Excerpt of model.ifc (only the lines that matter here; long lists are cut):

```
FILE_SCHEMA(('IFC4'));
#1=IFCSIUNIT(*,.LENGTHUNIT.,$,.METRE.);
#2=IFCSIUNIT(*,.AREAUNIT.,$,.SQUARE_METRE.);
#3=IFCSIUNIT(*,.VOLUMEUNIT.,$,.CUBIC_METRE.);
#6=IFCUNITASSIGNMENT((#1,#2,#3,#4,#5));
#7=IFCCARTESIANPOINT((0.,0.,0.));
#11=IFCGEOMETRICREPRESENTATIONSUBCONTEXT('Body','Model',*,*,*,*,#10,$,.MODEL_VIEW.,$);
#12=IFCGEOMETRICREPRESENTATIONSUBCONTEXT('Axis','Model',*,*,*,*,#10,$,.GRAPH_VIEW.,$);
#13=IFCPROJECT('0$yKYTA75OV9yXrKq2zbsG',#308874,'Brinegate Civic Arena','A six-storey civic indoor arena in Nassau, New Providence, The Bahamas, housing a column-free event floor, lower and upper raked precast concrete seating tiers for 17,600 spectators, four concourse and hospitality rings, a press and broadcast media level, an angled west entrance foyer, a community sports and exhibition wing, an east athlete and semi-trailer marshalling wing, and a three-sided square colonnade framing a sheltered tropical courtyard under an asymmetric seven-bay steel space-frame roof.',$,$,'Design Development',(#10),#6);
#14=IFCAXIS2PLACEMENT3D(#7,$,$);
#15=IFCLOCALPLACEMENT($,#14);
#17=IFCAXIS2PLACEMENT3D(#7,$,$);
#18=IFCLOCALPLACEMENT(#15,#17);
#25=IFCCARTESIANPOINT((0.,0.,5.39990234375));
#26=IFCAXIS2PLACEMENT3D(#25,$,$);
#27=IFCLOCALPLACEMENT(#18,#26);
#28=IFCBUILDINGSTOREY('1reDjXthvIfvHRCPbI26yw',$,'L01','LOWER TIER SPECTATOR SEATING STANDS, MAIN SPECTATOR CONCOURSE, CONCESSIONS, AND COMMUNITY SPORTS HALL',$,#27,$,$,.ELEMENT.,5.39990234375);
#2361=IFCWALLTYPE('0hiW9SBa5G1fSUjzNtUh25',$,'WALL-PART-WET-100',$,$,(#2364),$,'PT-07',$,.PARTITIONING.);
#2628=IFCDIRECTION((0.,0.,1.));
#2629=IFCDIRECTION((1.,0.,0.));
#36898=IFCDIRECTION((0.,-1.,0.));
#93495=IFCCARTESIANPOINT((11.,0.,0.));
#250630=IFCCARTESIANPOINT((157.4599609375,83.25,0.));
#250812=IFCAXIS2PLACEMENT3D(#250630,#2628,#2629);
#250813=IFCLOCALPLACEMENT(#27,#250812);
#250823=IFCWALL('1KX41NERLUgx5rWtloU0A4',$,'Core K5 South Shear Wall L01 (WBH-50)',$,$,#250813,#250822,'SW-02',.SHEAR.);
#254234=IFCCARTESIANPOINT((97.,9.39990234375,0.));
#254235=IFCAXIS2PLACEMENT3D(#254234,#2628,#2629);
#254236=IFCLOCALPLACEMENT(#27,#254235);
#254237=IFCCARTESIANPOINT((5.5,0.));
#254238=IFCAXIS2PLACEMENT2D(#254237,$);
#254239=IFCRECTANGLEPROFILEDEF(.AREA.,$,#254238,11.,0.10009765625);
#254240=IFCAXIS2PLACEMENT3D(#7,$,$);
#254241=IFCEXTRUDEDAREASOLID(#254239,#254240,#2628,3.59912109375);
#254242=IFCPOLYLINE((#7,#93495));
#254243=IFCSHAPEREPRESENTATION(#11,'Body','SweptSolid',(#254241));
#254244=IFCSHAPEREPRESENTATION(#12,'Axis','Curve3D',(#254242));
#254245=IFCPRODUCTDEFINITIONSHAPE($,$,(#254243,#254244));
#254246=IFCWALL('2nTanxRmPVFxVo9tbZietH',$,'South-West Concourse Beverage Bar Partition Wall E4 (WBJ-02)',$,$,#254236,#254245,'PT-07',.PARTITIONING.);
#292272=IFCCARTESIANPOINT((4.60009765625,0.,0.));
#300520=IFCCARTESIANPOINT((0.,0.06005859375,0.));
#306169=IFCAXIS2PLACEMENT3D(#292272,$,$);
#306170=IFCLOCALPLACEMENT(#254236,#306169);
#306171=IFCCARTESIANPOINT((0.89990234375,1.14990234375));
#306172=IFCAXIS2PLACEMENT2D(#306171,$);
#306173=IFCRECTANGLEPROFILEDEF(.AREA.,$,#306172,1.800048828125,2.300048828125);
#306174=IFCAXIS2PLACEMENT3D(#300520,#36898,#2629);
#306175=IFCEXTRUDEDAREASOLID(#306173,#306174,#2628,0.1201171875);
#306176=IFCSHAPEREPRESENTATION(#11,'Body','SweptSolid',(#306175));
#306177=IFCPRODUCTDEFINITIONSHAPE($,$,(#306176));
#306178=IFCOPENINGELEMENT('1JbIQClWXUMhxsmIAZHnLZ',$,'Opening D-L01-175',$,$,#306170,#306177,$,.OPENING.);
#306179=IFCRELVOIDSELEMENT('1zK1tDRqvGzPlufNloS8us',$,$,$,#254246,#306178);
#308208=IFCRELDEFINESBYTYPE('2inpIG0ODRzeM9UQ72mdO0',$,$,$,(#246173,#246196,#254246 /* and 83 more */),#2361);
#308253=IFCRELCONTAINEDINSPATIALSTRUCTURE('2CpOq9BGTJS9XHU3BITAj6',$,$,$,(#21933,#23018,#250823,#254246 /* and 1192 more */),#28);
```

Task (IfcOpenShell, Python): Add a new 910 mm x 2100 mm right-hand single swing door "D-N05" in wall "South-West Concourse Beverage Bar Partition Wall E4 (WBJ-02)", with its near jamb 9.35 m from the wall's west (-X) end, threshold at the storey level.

```python
import numpy as np
import ifcopenshell
import ifcopenshell.api.feature
import ifcopenshell.api.geometry
import ifcopenshell.api.root
import ifcopenshell.api.spatial
import ifcopenshell.geom
import ifcopenshell.util.element
import ifcopenshell.util.placement
import ifcopenshell.util.representation
import ifcopenshell.util.shape
import ifcopenshell.util.unit

model = ifcopenshell.open("model.ifc")
unit_scale = ifcopenshell.util.unit.calculate_unit_scale(model)
settings = ifcopenshell.geom.settings()


def volume(element):
    """Net volume in cubic metres, openings subtracted."""
    shape = ifcopenshell.geom.create_shape(settings, element)
    return ifcopenshell.util.shape.get_volume(shape.geometry)


wall = model.by_id(254246)
storey = ifcopenshell.util.element.get_container(wall, ifc_class="IfcBuildingStorey")
context = ifcopenshell.util.representation.get_context(model, "Model", "Body", "MODEL_VIEW")
before = volume(wall)

width, height, from_end, sill = 0.91, 2.1, 9.35, 0.0  # metres

# The wall runs along its own X axis, and the end named is its -X end.
wall_shape = ifcopenshell.geom.create_shape(settings, wall)
x, y, z = ifcopenshell.util.shape.get_vertices(wall_shape.geometry).T
start = x.min() + from_end
face, thickness = float(y.min()), float(y.max() - y.min())
wall_matrix = ifcopenshell.util.placement.get_local_placement(wall.ObjectPlacement)
level = ifcopenshell.util.placement.get_local_placement(storey.ObjectPlacement)[2, 3]


def in_wall(x, y):
    """Placement at x, y metres in the wall's axes, at sill height."""
    matrix = wall_matrix.copy()
    matrix[:, 3] = wall_matrix @ np.array([x / unit_scale, y / unit_scale, 0.0, 1.0])
    matrix[2, 3] = level + sill / unit_scale
    return matrix


# Opening: a box that overshoots both wall faces by 50 mm.
opening = ifcopenshell.api.root.create_entity(model, ifc_class="IfcOpeningElement", predefined_type="OPENING")
box = ifcopenshell.api.geometry.add_wall_representation(
    model, context=context, length=width, height=height, thickness=thickness + 0.1
)
ifcopenshell.api.geometry.assign_representation(model, product=opening, representation=box)
ifcopenshell.api.geometry.edit_object_placement(model, product=opening, matrix=in_wall(start, face - 0.05), is_si=False)
ifcopenshell.api.feature.add_feature(model, feature=opening, element=wall)

door = ifcopenshell.api.root.create_entity(model, ifc_class="IfcDoor", name="D-N05", predefined_type="DOOR")
door.OverallWidth, door.OverallHeight = width / unit_scale, height / unit_scale
door.OperationType = "SINGLE_SWING_RIGHT"
body = ifcopenshell.api.geometry.add_door_representation(
    model,
    context=context,
    overall_width=door.OverallWidth,
    overall_height=door.OverallHeight,
    operation_type="SINGLE_SWING_RIGHT",
    lining_properties={"LiningDepth": thickness / unit_scale, "ThresholdDepth": thickness / unit_scale},
)
ifcopenshell.api.geometry.assign_representation(model, product=door, representation=body)
ifcopenshell.api.spatial.assign_container(model, products=[door], relating_structure=storey)
ifcopenshell.api.feature.add_filling(model, opening=opening, element=door)

# The lining spans the wall, so the door starts at the wall face.
ifcopenshell.api.geometry.edit_object_placement(model, product=door, matrix=in_wall(start, face), is_si=False)

after = volume(wall)

print(f"wall volume {before:.3f} -> {after:.3f} m3")

model.write("model_updated.ifc")
```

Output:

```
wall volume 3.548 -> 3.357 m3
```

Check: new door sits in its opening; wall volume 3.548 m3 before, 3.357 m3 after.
